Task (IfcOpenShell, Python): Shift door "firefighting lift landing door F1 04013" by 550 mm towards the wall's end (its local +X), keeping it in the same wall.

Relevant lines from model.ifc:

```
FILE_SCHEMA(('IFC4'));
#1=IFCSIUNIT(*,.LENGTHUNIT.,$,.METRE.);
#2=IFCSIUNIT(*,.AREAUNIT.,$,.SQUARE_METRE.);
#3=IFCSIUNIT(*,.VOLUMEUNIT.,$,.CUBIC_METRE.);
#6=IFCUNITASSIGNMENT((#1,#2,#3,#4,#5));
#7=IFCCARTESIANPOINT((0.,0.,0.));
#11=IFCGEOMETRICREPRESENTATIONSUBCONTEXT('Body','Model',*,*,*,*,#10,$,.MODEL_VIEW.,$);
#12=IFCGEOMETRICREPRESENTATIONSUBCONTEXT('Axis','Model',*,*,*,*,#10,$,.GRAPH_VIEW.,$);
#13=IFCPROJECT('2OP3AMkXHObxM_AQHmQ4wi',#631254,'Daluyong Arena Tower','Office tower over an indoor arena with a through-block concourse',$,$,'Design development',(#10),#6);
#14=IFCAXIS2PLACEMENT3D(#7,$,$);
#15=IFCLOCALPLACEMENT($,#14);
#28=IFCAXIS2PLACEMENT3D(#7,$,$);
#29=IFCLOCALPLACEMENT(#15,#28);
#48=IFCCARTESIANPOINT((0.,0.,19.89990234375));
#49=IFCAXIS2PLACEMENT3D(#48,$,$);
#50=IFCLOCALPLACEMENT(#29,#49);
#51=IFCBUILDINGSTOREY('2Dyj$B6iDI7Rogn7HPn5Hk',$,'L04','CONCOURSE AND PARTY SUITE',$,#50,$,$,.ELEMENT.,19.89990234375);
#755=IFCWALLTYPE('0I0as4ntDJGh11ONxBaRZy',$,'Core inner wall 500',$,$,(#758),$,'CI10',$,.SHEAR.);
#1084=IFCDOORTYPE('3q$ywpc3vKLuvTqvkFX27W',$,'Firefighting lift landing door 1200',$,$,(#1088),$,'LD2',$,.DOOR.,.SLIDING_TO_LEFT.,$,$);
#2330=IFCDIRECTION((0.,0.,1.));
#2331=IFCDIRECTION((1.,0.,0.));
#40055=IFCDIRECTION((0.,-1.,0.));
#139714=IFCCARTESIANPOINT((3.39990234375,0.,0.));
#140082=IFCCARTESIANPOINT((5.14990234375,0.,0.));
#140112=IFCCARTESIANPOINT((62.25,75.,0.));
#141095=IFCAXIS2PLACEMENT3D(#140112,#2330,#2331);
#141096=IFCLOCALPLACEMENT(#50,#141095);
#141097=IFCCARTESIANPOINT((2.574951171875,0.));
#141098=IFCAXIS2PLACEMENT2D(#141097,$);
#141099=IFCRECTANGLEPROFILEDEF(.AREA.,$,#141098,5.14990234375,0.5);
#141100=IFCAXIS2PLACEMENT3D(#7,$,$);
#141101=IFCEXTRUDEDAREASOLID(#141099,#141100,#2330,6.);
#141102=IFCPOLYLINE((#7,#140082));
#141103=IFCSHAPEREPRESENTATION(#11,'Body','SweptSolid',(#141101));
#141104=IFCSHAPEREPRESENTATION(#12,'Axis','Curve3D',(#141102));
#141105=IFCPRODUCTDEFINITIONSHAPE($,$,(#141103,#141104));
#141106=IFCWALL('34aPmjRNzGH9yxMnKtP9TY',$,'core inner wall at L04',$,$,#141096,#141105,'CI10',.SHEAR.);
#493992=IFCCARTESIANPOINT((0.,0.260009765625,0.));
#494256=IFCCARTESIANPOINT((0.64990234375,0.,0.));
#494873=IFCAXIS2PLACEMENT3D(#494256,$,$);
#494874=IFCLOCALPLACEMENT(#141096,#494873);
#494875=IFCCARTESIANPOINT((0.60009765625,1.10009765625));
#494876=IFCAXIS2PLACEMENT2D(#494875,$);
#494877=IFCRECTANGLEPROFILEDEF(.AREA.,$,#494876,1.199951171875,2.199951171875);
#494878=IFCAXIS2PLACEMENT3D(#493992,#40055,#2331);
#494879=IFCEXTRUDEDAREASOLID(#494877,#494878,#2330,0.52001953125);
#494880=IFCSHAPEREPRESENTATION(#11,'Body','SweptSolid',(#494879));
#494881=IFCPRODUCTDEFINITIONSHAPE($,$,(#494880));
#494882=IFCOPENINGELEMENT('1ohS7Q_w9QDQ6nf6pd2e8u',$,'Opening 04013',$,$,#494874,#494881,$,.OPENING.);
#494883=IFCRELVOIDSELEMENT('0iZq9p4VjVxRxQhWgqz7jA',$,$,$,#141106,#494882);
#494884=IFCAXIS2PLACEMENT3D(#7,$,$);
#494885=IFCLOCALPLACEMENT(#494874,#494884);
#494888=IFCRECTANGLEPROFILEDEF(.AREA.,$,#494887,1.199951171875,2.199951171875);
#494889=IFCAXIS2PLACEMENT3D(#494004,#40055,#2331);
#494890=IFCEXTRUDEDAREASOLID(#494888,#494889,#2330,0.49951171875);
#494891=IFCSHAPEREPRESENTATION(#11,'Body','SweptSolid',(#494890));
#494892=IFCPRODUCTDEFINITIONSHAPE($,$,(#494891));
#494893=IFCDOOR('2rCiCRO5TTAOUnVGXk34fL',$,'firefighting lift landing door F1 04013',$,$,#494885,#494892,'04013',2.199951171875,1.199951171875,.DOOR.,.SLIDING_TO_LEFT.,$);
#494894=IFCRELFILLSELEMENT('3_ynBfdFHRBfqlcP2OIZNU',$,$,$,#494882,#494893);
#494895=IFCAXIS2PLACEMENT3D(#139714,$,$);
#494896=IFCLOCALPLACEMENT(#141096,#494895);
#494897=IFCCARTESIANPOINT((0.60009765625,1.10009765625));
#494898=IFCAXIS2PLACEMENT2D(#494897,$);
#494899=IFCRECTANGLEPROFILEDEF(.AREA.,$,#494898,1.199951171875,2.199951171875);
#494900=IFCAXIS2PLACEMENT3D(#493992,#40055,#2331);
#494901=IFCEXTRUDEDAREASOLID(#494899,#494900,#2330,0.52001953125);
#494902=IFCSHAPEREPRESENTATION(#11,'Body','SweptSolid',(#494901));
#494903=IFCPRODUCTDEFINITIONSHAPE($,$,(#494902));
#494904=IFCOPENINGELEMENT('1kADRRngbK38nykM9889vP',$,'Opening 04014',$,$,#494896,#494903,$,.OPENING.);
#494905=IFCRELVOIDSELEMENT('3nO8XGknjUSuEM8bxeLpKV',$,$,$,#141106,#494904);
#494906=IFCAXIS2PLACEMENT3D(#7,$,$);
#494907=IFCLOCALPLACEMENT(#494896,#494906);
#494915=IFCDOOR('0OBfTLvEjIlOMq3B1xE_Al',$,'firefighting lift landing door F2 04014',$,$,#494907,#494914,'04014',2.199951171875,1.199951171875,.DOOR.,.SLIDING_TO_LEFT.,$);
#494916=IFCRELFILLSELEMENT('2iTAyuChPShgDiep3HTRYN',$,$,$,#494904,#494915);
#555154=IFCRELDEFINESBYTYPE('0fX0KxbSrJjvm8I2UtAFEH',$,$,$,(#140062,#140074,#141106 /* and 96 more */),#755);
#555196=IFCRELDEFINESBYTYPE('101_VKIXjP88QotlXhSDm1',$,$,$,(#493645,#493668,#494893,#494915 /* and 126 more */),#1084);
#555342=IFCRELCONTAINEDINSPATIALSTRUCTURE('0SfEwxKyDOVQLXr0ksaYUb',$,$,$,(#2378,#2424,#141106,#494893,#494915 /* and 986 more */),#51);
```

```python
import ifcopenshell
import ifcopenshell.api.geometry
import ifcopenshell.util.placement
import ifcopenshell.util.unit

model = ifcopenshell.open("model.ifc")
unit_scale = ifcopenshell.util.unit.calculate_unit_scale(model)

door = model.by_guid("2rCiCRO5TTAOUnVGXk34fL")
opening = door.FillsVoids[0].RelatingOpeningElement
wall = opening.VoidsElements[0].RelatingBuildingElement

wall_matrix = ifcopenshell.util.placement.get_local_placement(wall.ObjectPlacement)
shift = wall_matrix[:3, 0] * 0.55 / unit_scale
before = ifcopenshell.util.placement.get_local_placement(door.ObjectPlacement)[:3, 3].copy()

# The door is placed relative to its opening, so it follows when the opening moves.
matrix = ifcopenshell.util.placement.get_local_placement(opening.ObjectPlacement)
matrix[:3, 3] += shift
ifcopenshell.api.geometry.edit_object_placement(
    model, product=opening, matrix=matrix, is_si=False, should_transform_children=True
)

after = ifcopenshell.util.placement.get_local_placement(door.ObjectPlacement)[:3, 3]
print("door moved by", (after - before).round(3) + 0.0)

model.write("model-out.ifc")
```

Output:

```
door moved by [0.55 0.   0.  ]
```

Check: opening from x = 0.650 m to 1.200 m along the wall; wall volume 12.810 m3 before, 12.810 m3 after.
